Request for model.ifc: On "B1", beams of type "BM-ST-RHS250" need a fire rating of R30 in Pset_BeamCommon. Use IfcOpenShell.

First a look at what the model holds.

```python
import ifcopenshell
import ifcopenshell.util.element

model = ifcopenshell.open("model.ifc")
print(model.schema)
storey = next(s for s in model.by_type("IfcBuildingStorey") if s.Name == "B1")
beams = [e for e in ifcopenshell.util.element.get_decomposition(storey) if e.is_a("IfcBeam")]
seen = {}
for e in beams:
    element_type = ifcopenshell.util.element.get_type(e)
    key = (element_type.Name if element_type != e and element_type else None, ifcopenshell.util.element.get_pset(e, "Pset_BeamCommon", "FireRating"))
    seen[key] = seen.get(key, 0) + 1
for (name, value), count in sorted(seen.items(), key=str):
    print(count, "x", name, "|", value)
```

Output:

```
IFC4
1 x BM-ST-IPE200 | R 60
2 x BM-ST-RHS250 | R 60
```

```python
import ifcopenshell
import ifcopenshell.api.pset
import ifcopenshell.util.element

model = ifcopenshell.open("model.ifc")

storey = next(s for s in model.by_type("IfcBuildingStorey") if s.Name == "B1")
beams = [e for e in ifcopenshell.util.element.get_decomposition(storey) if e.is_a("IfcBeam")]

count = 0
for e in beams:
    element_type = ifcopenshell.util.element.get_type(e)
    if element_type in (None, e) or element_type.Name != "BM-ST-RHS250":
        continue
    # add_pset returns the element's existing set when there is one.
    pset = ifcopenshell.api.pset.add_pset(model, product=e, name="Pset_BeamCommon")
    ifcopenshell.api.pset.edit_pset(model, pset=pset, properties={"FireRating": "R30"})
    count += 1

print(count, "beams updated")

model.write("model_updated.ifc")
```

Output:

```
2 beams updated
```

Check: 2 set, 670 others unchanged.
